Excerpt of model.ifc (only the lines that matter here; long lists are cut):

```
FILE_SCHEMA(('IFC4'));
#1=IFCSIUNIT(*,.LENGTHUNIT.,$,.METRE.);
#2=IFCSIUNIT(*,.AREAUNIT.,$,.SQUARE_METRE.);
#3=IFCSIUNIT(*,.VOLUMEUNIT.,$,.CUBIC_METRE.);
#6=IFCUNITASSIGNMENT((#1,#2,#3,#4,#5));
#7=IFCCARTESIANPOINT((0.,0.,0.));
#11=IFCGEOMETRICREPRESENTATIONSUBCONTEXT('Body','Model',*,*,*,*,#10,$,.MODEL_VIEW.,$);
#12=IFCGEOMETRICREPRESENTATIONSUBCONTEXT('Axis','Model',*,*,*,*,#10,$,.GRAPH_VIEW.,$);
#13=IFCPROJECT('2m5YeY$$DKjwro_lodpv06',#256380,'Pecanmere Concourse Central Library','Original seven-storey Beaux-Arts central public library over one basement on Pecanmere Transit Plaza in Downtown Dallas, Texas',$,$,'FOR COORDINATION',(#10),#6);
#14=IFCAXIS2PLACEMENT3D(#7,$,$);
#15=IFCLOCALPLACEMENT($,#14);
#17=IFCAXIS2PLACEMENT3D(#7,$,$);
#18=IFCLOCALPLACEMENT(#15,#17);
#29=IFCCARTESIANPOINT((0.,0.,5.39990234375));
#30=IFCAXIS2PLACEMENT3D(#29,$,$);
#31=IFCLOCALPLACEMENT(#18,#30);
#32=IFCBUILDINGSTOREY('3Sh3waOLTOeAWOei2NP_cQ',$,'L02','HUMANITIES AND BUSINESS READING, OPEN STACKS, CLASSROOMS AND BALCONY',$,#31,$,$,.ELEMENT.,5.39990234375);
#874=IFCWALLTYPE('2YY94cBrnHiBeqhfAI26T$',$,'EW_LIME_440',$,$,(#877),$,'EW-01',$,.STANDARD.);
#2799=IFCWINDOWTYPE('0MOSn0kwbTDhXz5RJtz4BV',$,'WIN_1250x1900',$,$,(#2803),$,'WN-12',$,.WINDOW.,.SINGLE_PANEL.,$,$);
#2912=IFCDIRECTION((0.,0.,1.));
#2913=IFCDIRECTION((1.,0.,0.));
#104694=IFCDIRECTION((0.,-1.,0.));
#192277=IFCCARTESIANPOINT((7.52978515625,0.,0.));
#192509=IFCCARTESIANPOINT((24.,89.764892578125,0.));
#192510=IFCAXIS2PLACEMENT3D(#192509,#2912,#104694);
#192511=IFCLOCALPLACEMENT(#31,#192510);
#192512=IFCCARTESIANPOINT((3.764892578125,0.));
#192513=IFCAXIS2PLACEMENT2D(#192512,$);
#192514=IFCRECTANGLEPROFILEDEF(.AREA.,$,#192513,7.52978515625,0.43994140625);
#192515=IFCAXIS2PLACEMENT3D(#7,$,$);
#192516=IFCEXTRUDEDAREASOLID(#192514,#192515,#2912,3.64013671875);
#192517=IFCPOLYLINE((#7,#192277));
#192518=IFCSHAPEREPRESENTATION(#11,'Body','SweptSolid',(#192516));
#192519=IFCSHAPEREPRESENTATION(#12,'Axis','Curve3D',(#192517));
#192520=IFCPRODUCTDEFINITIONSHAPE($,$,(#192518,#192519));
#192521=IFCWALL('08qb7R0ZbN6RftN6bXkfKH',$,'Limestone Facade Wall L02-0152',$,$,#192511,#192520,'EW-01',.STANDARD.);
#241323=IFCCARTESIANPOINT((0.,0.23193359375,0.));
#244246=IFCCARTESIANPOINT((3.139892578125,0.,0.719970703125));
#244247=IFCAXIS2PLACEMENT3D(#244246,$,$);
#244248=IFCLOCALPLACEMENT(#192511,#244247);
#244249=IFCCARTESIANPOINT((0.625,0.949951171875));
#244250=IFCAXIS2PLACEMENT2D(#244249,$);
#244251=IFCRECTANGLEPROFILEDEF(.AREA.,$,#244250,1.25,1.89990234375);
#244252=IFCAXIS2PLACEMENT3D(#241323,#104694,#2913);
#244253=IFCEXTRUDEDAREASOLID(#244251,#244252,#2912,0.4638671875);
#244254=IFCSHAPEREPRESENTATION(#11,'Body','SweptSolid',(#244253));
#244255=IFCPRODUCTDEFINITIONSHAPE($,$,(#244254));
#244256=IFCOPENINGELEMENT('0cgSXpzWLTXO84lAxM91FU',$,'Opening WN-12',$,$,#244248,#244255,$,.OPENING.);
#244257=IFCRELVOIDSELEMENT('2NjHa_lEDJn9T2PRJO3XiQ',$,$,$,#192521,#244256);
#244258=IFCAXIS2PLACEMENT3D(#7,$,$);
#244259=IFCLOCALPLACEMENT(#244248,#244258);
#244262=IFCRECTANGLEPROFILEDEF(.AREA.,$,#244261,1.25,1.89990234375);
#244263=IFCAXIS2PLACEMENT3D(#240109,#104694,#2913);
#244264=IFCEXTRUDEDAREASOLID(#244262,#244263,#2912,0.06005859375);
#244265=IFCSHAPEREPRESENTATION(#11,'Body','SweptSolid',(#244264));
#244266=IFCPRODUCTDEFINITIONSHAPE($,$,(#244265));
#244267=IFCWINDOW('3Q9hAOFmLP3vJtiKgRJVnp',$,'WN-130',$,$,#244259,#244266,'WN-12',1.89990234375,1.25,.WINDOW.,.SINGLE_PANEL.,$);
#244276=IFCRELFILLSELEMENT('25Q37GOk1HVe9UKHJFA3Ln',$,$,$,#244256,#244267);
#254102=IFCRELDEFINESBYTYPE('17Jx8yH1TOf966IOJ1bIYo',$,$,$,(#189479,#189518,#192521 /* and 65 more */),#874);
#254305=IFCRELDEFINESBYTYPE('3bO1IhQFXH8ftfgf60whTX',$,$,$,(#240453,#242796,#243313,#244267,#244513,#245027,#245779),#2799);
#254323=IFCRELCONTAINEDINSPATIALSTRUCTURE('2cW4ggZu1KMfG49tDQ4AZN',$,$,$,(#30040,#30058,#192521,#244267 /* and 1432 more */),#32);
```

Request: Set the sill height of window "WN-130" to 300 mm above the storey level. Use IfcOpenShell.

```python
import numpy as np
import ifcopenshell
import ifcopenshell.api.geometry
import ifcopenshell.geom
import ifcopenshell.util.element
import ifcopenshell.util.placement
import ifcopenshell.util.shape
import ifcopenshell.util.unit

model = ifcopenshell.open("model.ifc")
unit_scale = ifcopenshell.util.unit.calculate_unit_scale(model)

window = model.by_id(244267)
opening = window.FillsVoids[0].RelatingOpeningElement
storey = ifcopenshell.util.element.get_container(window, ifc_class="IfcBuildingStorey")
level = ifcopenshell.util.placement.get_local_placement(storey.ObjectPlacement)[2, 3]

# The opening's origin need not be at the sill, so measure its lowest point.
shape = ifcopenshell.geom.create_shape(ifcopenshell.geom.settings(), opening)
bottom = ifcopenshell.util.shape.get_shape_bottom_elevation(shape, shape.geometry) / unit_scale
dz = level + 0.3 - bottom

shift = np.array([0.0, 0.0, dz])
# The window is placed relative to its opening, so it follows when the opening moves.
matrix = ifcopenshell.util.placement.get_local_placement(opening.ObjectPlacement)
matrix[:3, 3] += shift
ifcopenshell.api.geometry.edit_object_placement(
    model, product=opening, matrix=matrix, is_si=False, should_transform_children=True
)

print(f"moved by {dz * unit_scale:+.3f} m")

model.write("model_v2.ifc")
```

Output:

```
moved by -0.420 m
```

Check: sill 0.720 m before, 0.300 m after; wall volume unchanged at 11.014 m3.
